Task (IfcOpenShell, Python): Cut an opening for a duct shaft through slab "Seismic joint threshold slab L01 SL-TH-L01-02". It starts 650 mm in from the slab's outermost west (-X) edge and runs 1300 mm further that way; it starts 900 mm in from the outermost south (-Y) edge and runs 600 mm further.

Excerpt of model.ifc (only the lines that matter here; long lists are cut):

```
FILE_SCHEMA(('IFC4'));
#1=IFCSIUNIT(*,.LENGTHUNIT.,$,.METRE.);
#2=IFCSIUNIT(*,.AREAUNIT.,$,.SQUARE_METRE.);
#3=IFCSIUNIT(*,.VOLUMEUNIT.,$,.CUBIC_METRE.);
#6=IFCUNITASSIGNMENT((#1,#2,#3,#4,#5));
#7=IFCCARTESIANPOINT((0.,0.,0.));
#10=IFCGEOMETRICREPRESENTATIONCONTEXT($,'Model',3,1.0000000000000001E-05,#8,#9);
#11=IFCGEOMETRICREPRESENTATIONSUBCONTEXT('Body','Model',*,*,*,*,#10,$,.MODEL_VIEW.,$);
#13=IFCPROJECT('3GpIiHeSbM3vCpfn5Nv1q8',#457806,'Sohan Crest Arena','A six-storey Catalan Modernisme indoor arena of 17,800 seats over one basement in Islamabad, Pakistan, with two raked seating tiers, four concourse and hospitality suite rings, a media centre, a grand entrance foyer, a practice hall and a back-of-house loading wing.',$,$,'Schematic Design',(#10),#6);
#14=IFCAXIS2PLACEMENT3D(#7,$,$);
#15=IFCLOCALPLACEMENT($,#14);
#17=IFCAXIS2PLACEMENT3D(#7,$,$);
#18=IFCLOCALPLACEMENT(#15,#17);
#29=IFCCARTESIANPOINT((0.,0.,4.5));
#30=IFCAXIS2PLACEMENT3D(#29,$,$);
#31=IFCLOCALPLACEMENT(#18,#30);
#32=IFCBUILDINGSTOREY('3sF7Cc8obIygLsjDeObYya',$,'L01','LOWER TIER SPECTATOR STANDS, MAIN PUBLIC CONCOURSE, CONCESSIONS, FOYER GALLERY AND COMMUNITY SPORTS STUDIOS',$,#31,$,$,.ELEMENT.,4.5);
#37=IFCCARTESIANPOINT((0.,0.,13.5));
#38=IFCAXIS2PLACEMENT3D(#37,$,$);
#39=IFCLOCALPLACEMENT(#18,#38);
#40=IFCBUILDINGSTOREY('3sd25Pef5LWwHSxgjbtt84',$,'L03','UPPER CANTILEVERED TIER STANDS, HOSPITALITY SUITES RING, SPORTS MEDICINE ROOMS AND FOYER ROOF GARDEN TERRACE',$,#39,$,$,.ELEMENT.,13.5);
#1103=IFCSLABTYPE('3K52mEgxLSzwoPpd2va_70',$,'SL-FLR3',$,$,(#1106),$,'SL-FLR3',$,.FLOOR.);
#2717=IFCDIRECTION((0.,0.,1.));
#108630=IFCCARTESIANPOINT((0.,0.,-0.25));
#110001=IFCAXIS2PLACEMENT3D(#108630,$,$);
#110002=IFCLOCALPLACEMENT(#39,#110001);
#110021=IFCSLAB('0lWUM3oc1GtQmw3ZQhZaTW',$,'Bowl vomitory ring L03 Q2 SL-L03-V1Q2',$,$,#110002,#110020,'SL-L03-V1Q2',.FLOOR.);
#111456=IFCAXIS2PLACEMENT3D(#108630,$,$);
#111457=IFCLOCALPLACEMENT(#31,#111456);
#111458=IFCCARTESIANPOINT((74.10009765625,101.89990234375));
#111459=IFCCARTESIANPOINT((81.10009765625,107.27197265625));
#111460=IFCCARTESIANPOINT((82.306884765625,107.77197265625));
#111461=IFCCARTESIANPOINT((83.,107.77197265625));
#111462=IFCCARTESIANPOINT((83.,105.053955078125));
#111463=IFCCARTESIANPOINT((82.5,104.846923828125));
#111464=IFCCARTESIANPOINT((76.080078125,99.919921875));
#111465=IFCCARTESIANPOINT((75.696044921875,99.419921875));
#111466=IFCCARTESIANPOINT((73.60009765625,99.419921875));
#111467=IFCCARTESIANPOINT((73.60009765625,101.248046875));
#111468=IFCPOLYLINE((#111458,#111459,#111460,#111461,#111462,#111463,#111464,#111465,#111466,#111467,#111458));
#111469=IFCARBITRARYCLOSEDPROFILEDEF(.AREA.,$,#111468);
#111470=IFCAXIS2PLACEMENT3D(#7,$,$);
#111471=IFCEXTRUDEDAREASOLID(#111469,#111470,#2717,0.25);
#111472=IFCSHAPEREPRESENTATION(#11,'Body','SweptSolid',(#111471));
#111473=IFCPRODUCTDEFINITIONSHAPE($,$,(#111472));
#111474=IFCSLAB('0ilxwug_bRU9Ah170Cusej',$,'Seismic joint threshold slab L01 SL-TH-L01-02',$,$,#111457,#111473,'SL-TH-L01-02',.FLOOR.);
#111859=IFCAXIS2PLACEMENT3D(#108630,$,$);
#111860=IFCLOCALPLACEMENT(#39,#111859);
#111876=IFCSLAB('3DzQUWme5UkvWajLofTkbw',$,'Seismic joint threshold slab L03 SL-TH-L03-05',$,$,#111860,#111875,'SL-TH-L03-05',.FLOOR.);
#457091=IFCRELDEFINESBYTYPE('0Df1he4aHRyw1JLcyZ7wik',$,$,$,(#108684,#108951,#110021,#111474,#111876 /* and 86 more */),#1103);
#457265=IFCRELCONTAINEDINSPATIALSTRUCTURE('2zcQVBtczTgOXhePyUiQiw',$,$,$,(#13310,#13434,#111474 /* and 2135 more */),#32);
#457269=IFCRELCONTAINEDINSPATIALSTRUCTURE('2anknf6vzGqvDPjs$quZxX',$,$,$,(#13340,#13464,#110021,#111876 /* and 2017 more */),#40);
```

```python
import numpy as np
import ifcopenshell
import ifcopenshell.api.feature
import ifcopenshell.api.geometry
import ifcopenshell.api.root
import ifcopenshell.geom
import ifcopenshell.util.placement
import ifcopenshell.util.representation
import ifcopenshell.util.shape
import ifcopenshell.util.unit

model = ifcopenshell.open("model.ifc")
unit_scale = ifcopenshell.util.unit.calculate_unit_scale(model)
settings = ifcopenshell.geom.settings()


def volume(element):
    """Net volume in cubic metres, openings subtracted."""
    shape = ifcopenshell.geom.create_shape(settings, element)
    return ifcopenshell.util.shape.get_volume(shape.geometry)


slab = model.by_guid("0ilxwug_bRU9Ah170Cusej")
before = volume(slab)

# Extent in the slab's own axes, in metres. The edges named are its -X and -Y sides.
slab_shape = ifcopenshell.geom.create_shape(settings, slab)
vertices = ifcopenshell.util.shape.get_vertices(slab_shape.geometry)
x_min, y_min, bottom = vertices.min(axis=0)
top = vertices[:, 2].max()

opening = ifcopenshell.api.root.create_entity(model, ifc_class="IfcOpeningElement", name="Duct shaft opening", predefined_type="OPENING")
context = ifcopenshell.util.representation.get_context(model, "Model", "Body", "MODEL_VIEW")
width, depth = 1.3, 0.6
outline = [(0.0, 0.0), (width, 0.0), (width, depth), (0.0, depth), (0.0, 0.0)]
# Overshoot both faces by 50 mm so the cut is clean.
shape = ifcopenshell.api.geometry.add_slab_representation(
    model, context=context, depth=top - bottom + 0.1, polyline=outline
)
ifcopenshell.api.geometry.assign_representation(model, product=opening, representation=shape)

matrix = ifcopenshell.util.placement.get_local_placement(slab.ObjectPlacement)
matrix[:, 3] = matrix @ np.append(np.array([x_min + 0.65, y_min + 0.9, bottom - 0.05]) / unit_scale, 1.0)
ifcopenshell.api.geometry.edit_object_placement(model, product=opening, matrix=matrix, is_si=False)
ifcopenshell.api.feature.add_feature(model, feature=opening, element=slab)

after = volume(slab)

print(f"slab volume {before:.3f} -> {after:.3f} m3")

model.write("model_rev.ifc")
```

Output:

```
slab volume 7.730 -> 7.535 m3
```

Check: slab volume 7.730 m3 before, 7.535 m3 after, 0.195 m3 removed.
